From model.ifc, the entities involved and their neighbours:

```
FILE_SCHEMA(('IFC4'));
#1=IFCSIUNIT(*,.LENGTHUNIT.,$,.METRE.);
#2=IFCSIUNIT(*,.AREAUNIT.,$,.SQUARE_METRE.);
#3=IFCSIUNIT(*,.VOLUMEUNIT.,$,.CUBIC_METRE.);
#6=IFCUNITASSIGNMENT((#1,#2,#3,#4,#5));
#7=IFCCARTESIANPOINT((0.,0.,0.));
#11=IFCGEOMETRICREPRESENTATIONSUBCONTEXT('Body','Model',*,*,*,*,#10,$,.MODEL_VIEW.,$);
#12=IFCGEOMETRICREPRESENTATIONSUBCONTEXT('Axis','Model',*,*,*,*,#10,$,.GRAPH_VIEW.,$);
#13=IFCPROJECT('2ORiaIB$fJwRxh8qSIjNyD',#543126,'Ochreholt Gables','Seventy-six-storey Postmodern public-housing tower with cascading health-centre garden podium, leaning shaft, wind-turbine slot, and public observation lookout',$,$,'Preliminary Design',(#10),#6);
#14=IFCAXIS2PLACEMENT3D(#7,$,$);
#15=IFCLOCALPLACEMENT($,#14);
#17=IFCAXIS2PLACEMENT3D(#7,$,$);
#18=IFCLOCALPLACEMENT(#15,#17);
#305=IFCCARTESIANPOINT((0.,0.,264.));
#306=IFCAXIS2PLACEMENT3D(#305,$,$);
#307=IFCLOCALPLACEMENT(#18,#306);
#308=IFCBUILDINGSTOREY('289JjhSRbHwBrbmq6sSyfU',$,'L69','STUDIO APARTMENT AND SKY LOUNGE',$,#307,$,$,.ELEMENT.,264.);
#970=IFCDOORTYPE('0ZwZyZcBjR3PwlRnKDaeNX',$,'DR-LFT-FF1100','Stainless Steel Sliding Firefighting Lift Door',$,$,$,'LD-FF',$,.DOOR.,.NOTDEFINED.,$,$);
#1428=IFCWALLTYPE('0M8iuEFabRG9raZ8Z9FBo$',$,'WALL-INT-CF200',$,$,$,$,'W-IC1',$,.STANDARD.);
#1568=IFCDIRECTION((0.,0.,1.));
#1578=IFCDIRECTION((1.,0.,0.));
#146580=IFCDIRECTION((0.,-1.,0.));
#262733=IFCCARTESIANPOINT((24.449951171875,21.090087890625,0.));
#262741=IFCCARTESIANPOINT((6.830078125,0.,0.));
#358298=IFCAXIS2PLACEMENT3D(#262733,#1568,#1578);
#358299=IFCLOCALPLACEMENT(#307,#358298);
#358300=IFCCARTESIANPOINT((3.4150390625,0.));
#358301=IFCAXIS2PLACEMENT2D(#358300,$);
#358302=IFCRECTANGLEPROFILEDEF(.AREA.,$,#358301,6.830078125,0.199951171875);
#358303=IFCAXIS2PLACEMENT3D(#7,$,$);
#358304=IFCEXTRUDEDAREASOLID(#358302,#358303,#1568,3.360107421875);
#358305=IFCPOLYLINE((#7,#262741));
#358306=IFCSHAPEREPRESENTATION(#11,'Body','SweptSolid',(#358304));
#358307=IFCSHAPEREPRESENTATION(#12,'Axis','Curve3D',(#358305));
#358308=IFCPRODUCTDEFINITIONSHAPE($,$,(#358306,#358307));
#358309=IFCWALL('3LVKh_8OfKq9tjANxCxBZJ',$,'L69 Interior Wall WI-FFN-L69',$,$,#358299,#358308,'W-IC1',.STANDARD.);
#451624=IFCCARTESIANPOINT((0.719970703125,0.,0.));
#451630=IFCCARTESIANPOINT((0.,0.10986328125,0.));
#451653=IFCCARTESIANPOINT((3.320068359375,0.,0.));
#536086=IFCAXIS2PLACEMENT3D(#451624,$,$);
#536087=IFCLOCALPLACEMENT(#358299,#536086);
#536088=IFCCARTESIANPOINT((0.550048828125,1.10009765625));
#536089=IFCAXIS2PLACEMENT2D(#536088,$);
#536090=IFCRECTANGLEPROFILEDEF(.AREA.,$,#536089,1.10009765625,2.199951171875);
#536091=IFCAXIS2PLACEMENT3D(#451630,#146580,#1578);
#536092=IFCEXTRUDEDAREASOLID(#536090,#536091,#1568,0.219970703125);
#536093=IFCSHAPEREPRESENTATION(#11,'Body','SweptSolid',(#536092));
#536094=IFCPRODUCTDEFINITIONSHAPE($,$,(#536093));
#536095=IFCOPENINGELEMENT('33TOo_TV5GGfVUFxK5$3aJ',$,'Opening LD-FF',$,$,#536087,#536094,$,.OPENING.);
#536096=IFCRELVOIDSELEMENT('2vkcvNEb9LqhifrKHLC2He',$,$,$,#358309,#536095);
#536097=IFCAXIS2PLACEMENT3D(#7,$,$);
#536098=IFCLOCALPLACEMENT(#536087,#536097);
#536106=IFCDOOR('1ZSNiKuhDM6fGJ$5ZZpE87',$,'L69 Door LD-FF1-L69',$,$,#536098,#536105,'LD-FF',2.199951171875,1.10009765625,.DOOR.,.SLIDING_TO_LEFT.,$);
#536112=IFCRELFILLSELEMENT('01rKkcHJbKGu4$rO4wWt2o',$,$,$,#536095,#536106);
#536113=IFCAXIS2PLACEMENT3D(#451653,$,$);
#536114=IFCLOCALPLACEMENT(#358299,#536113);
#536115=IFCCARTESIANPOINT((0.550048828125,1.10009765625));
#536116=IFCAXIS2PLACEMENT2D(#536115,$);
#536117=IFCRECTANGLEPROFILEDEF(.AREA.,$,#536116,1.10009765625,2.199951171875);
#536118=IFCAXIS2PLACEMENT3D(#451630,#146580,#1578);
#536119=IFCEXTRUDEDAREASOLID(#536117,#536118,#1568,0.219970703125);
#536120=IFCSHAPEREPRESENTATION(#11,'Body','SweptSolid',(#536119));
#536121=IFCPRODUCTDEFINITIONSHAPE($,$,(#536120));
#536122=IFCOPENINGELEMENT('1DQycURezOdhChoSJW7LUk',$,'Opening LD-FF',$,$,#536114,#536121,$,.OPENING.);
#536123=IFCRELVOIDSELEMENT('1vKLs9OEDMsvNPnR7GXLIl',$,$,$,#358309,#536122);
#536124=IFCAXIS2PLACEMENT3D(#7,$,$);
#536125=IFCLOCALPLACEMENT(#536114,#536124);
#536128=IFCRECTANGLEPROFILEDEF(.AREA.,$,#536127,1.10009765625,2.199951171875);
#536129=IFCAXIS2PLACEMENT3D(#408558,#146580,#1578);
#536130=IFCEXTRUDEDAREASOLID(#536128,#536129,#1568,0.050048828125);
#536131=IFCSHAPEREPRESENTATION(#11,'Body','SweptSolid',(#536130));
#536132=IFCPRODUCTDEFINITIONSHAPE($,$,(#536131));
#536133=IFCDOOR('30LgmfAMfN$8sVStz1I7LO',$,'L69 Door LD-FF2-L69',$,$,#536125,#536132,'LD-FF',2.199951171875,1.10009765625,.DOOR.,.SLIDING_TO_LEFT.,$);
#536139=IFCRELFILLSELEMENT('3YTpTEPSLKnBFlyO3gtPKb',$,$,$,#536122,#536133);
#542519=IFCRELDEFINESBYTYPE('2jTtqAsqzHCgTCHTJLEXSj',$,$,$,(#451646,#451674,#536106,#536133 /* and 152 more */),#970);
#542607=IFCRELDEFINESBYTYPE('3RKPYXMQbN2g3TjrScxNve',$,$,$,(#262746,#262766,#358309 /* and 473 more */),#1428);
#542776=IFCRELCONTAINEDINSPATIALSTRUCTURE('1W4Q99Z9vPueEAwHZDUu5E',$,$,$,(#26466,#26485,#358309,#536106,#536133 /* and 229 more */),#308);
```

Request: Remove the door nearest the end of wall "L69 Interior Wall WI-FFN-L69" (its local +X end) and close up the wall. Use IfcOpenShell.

```python
import ifcopenshell
import ifcopenshell.api.feature
import ifcopenshell.api.root
import ifcopenshell.geom
import ifcopenshell.util.shape

model = ifcopenshell.open("model.ifc")
settings = ifcopenshell.geom.settings()


def volume(element):
    """Net volume in cubic metres, openings subtracted."""
    shape = ifcopenshell.geom.create_shape(settings, element)
    return ifcopenshell.util.shape.get_volume(shape.geometry)


door = model.by_guid("30LgmfAMfN$8sVStz1I7LO")
opening = door.FillsVoids[0].RelatingOpeningElement
wall = opening.VoidsElements[0].RelatingBuildingElement
before = volume(wall)

ifcopenshell.api.root.remove_product(model, product=door)
ifcopenshell.api.feature.remove_feature(model, feature=opening)

after = volume(wall)

print(f"wall volume {before:.3f} -> {after:.3f} m3")

model.write("model_v2.ifc")
```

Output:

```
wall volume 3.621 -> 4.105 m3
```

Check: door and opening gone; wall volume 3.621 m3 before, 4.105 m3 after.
